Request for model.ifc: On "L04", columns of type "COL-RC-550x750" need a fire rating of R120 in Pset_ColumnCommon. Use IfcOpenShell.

First a look at what the model holds.

```python
import ifcopenshell
import ifcopenshell.util.element

model = ifcopenshell.open("model.ifc")
print(model.schema)
storey = next(s for s in model.by_type("IfcBuildingStorey") if s.Name == "L04")
columns = [e for e in ifcopenshell.util.element.get_decomposition(storey) if e.is_a("IfcColumn")]
seen = {}
for e in columns:
    element_type = ifcopenshell.util.element.get_type(e)
    key = (element_type.Name if element_type != e and element_type else None, ifcopenshell.util.element.get_pset(e, "Pset_ColumnCommon", "FireRating"))
    seen[key] = seen.get(key, 0) + 1
for (name, value), count in sorted(seen.items(), key=str):
    print(count, "x", name, "|", value)
```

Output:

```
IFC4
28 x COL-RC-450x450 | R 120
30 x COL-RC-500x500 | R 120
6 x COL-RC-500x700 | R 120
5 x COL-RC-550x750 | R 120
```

```python
import ifcopenshell
import ifcopenshell.api.pset
import ifcopenshell.util.element

model = ifcopenshell.open("model.ifc")

storey = next(s for s in model.by_type("IfcBuildingStorey") if s.Name == "L04")
columns = [e for e in ifcopenshell.util.element.get_decomposition(storey) if e.is_a("IfcColumn")]

count = 0
for e in columns:
    element_type = ifcopenshell.util.element.get_type(e)
    if element_type in (None, e) or element_type.Name != "COL-RC-550x750":
        continue
    # add_pset returns the element's existing set when there is one.
    pset = ifcopenshell.api.pset.add_pset(model, product=e, name="Pset_ColumnCommon")
    ifcopenshell.api.pset.edit_pset(model, pset=pset, properties={"FireRating": "R120"})
    count += 1

print(count, "columns updated")

model.write("model_edited.ifc")
```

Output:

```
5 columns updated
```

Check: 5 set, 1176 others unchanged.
